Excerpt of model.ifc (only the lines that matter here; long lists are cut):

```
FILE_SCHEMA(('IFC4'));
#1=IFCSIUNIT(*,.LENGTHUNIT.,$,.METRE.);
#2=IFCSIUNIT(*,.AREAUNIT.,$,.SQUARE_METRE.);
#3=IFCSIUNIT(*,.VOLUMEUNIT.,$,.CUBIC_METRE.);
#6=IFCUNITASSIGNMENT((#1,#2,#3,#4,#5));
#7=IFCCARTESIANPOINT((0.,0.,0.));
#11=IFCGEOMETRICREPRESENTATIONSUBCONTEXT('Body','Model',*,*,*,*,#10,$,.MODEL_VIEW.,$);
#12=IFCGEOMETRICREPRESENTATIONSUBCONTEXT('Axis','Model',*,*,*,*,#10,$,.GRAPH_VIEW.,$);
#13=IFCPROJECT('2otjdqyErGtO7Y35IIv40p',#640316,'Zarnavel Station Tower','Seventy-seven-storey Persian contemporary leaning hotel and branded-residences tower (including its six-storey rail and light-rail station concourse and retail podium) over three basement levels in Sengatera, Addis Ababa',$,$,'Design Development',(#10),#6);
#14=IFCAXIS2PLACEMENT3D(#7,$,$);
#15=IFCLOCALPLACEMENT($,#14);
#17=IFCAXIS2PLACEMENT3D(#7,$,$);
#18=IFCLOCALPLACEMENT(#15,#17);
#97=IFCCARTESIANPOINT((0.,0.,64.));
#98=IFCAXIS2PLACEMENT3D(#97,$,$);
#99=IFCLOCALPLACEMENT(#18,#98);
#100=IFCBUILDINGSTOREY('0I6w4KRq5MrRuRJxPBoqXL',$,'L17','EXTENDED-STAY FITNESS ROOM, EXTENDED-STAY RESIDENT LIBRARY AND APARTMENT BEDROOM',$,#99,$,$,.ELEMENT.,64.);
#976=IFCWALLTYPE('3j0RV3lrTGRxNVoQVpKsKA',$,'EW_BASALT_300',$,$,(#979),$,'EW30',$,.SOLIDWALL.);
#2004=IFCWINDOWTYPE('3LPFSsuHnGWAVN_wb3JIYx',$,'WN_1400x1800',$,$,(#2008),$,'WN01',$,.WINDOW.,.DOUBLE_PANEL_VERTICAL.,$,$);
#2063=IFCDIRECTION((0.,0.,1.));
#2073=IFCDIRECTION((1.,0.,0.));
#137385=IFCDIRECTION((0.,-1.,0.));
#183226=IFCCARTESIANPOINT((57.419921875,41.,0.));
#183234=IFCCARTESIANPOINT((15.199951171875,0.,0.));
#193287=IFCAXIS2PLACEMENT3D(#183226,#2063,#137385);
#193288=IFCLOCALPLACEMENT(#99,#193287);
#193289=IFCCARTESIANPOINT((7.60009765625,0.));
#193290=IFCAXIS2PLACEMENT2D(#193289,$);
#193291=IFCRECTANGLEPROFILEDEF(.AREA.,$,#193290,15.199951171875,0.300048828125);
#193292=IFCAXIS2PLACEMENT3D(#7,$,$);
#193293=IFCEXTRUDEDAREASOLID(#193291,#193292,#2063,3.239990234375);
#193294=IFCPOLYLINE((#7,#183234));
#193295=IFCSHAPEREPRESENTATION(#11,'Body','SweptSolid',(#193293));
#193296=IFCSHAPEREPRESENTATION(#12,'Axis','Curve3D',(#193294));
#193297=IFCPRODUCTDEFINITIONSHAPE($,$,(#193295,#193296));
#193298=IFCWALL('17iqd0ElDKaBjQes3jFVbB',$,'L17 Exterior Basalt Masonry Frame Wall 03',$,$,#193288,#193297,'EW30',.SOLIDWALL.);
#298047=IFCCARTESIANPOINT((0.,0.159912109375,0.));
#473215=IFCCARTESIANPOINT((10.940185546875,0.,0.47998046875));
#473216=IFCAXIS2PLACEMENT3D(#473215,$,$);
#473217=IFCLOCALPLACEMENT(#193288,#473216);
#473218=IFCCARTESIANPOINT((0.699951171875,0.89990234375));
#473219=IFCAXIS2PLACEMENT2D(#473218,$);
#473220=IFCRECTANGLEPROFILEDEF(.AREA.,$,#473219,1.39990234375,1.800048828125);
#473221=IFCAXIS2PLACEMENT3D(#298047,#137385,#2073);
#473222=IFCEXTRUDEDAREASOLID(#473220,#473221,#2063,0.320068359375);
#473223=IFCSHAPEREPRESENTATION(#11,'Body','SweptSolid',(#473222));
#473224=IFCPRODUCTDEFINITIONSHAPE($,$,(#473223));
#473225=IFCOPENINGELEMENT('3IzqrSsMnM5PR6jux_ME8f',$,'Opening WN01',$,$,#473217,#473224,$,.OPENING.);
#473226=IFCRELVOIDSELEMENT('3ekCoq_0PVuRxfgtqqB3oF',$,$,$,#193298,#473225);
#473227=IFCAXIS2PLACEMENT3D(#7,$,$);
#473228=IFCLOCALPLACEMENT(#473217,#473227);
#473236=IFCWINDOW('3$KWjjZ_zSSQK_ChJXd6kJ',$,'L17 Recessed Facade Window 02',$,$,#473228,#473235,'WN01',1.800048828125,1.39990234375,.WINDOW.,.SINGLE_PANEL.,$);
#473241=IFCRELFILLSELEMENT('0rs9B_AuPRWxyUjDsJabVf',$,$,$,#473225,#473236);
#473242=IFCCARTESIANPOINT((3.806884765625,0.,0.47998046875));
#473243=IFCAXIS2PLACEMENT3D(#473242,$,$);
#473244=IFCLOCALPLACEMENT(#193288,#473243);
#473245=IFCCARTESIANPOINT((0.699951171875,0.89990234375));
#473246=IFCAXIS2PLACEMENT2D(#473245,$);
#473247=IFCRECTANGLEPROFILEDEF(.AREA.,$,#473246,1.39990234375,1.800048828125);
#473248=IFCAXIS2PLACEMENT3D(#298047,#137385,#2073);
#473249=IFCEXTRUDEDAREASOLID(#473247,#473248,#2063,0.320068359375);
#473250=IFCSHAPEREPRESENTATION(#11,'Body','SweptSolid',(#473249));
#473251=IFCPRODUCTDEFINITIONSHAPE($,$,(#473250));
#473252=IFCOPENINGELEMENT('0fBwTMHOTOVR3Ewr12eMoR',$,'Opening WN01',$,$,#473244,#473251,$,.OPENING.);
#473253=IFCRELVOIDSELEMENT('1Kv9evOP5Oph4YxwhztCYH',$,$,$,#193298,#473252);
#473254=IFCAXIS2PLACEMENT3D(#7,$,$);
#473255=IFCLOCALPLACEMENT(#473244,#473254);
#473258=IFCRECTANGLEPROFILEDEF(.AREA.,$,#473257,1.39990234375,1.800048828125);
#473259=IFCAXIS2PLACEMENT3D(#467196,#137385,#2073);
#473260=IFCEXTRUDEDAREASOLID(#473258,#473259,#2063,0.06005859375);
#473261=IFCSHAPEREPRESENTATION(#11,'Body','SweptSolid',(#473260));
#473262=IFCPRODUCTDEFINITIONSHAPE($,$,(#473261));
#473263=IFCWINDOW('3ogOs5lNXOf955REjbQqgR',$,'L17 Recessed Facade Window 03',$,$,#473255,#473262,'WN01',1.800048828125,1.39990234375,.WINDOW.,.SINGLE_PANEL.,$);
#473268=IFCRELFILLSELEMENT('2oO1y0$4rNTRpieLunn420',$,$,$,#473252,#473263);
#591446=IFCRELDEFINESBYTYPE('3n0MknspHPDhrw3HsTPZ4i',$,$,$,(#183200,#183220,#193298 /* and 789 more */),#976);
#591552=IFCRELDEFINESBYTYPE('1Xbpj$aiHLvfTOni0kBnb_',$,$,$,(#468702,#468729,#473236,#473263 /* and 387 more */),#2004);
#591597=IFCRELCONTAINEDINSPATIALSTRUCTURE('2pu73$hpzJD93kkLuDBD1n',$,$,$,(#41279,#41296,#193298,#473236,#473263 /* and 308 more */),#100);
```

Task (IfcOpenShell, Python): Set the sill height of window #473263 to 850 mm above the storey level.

```python
import numpy as np
import ifcopenshell
import ifcopenshell.api.geometry
import ifcopenshell.geom
import ifcopenshell.util.element
import ifcopenshell.util.placement
import ifcopenshell.util.shape
import ifcopenshell.util.unit

model = ifcopenshell.open("model.ifc")
unit_scale = ifcopenshell.util.unit.calculate_unit_scale(model)

window = model.by_id(473263)
opening = window.FillsVoids[0].RelatingOpeningElement
storey = ifcopenshell.util.element.get_container(window, ifc_class="IfcBuildingStorey")
level = ifcopenshell.util.placement.get_local_placement(storey.ObjectPlacement)[2, 3]

# The opening's origin need not be at the sill, so measure its lowest point.
shape = ifcopenshell.geom.create_shape(ifcopenshell.geom.settings(), opening)
bottom = ifcopenshell.util.shape.get_shape_bottom_elevation(shape, shape.geometry) / unit_scale
dz = level + 0.85 / unit_scale - bottom

shift = np.array([0.0, 0.0, dz])
# The window is placed relative to its opening, so it follows when the opening moves.
matrix = ifcopenshell.util.placement.get_local_placement(opening.ObjectPlacement)
matrix[:3, 3] += shift
ifcopenshell.api.geometry.edit_object_placement(
    model, product=opening, matrix=matrix, is_si=False, should_transform_children=True
)

print(f"moved by {dz * unit_scale:+.3f} m")

model.write("model_updated.ifc")
```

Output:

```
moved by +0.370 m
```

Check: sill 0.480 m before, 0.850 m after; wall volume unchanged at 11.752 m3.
